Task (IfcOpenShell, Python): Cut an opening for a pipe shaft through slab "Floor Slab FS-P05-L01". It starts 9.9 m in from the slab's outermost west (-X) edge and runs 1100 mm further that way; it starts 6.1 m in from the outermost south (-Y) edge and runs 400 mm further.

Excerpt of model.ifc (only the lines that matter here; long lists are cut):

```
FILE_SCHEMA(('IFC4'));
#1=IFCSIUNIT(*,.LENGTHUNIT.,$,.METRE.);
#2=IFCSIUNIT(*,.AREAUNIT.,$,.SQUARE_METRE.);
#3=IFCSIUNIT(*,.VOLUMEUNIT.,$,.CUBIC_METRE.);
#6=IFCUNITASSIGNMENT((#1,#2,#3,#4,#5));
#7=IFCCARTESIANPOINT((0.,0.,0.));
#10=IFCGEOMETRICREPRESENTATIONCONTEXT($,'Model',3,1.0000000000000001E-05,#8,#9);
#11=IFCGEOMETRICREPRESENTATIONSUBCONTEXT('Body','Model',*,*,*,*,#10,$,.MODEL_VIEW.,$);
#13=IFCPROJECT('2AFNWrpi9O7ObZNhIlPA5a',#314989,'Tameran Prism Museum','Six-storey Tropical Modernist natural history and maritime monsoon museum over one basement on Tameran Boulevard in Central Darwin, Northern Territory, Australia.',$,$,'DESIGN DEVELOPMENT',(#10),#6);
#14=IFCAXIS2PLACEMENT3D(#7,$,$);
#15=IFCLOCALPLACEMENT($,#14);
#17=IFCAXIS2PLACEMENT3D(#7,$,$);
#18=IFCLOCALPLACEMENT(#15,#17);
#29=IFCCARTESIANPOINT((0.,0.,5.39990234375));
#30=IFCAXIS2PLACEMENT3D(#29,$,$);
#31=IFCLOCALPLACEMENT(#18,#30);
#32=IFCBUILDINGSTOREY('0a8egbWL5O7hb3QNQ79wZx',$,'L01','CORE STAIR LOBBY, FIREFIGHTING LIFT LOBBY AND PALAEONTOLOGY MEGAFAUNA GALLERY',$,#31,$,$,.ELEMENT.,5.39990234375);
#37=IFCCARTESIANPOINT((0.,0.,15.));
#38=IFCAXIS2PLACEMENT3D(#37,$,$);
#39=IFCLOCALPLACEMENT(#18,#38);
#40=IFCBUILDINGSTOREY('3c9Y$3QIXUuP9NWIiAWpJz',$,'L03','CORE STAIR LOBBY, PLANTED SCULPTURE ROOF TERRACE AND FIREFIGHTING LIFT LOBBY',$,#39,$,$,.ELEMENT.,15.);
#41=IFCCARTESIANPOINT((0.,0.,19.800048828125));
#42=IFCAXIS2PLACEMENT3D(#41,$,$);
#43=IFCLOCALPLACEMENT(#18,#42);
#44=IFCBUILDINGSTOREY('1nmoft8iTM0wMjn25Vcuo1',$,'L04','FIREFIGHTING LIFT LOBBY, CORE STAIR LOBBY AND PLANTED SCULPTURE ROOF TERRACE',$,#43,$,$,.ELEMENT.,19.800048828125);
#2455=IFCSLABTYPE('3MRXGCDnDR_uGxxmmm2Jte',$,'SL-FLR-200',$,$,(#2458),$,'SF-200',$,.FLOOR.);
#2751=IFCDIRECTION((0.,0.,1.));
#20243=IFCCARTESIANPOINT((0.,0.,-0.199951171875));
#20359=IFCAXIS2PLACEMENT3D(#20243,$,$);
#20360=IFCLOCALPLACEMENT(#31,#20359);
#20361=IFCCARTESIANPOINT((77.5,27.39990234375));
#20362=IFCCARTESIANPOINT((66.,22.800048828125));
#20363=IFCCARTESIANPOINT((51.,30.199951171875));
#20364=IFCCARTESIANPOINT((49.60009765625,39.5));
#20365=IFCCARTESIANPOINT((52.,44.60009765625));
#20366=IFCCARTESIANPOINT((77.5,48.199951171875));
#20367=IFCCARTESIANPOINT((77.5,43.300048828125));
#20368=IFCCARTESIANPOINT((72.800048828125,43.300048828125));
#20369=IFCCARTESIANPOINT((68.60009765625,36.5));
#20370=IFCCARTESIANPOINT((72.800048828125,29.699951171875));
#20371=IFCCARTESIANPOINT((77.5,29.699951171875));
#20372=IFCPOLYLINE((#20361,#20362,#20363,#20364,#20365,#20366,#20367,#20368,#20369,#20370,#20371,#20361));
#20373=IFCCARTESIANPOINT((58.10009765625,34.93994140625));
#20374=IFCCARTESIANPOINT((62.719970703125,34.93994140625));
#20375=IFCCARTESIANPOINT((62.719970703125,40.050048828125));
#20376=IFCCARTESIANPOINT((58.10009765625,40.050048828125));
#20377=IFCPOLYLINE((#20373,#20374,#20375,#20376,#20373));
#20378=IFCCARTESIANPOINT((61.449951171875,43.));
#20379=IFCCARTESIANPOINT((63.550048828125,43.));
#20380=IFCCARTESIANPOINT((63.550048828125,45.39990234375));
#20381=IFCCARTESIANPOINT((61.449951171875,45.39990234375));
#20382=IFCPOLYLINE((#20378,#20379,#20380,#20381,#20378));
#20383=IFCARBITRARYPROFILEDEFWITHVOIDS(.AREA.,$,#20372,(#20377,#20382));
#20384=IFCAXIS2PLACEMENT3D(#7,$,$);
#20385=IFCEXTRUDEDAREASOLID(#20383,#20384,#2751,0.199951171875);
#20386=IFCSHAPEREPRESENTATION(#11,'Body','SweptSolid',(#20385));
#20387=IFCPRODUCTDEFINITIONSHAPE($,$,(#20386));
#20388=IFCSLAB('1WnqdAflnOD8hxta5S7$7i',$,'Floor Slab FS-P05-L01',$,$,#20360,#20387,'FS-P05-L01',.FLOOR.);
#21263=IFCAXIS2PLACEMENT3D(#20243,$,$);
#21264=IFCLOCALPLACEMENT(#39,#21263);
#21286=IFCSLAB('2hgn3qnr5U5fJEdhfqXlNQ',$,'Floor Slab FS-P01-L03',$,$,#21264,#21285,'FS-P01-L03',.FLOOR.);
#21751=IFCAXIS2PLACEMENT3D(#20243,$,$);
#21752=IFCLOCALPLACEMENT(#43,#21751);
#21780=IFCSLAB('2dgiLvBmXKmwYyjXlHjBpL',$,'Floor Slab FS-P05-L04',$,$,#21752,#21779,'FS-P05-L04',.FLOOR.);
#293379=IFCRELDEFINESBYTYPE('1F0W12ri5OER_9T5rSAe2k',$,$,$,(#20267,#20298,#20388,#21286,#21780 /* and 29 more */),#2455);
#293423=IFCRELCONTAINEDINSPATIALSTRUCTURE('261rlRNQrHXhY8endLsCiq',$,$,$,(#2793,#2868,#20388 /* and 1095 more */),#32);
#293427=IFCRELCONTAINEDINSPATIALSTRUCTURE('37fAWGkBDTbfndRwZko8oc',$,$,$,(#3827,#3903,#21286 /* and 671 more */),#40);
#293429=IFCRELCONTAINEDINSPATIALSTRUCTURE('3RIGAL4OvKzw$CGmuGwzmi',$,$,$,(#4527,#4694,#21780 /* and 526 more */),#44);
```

```python
import numpy as np
import ifcopenshell
import ifcopenshell.api.feature
import ifcopenshell.api.geometry
import ifcopenshell.api.root
import ifcopenshell.geom
import ifcopenshell.util.placement
import ifcopenshell.util.representation
import ifcopenshell.util.shape
import ifcopenshell.util.unit

model = ifcopenshell.open("model.ifc")
unit_scale = ifcopenshell.util.unit.calculate_unit_scale(model)
settings = ifcopenshell.geom.settings()


def volume(element):
    """Net volume in cubic metres, openings subtracted."""
    shape = ifcopenshell.geom.create_shape(settings, element)
    return ifcopenshell.util.shape.get_volume(shape.geometry)


slab = model.by_guid("1WnqdAflnOD8hxta5S7$7i")
before = volume(slab)

# Extent in the slab's own axes, in metres. The edges named are its -X and -Y sides.
slab_shape = ifcopenshell.geom.create_shape(settings, slab)
vertices = ifcopenshell.util.shape.get_vertices(slab_shape.geometry)
x_min, y_min, bottom = vertices.min(axis=0)
top = vertices[:, 2].max()

opening = ifcopenshell.api.root.create_entity(model, ifc_class="IfcOpeningElement", name="Pipe shaft opening", predefined_type="OPENING")
context = ifcopenshell.util.representation.get_context(model, "Model", "Body", "MODEL_VIEW")
width, depth = 1.1, 0.4
outline = [(0.0, 0.0), (width, 0.0), (width, depth), (0.0, depth), (0.0, 0.0)]
# Overshoot both faces by 50 mm so the cut is clean.
shape = ifcopenshell.api.geometry.add_slab_representation(
    model, context=context, depth=top - bottom + 0.1, polyline=outline
)
ifcopenshell.api.geometry.assign_representation(model, product=opening, representation=shape)

matrix = ifcopenshell.util.placement.get_local_placement(slab.ObjectPlacement)
matrix[:, 3] = matrix @ np.append(np.array([x_min + 9.9, y_min + 6.1, bottom - 0.05]) / unit_scale, 1.0)
ifcopenshell.api.geometry.edit_object_placement(model, product=opening, matrix=matrix, is_si=False)
ifcopenshell.api.feature.add_feature(model, feature=opening, element=slab)

after = volume(slab)

print(f"slab volume {before:.3f} -> {after:.3f} m3")

model.write("model_rev.ifc")
```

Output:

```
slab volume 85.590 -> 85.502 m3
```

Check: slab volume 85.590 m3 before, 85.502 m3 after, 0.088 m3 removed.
